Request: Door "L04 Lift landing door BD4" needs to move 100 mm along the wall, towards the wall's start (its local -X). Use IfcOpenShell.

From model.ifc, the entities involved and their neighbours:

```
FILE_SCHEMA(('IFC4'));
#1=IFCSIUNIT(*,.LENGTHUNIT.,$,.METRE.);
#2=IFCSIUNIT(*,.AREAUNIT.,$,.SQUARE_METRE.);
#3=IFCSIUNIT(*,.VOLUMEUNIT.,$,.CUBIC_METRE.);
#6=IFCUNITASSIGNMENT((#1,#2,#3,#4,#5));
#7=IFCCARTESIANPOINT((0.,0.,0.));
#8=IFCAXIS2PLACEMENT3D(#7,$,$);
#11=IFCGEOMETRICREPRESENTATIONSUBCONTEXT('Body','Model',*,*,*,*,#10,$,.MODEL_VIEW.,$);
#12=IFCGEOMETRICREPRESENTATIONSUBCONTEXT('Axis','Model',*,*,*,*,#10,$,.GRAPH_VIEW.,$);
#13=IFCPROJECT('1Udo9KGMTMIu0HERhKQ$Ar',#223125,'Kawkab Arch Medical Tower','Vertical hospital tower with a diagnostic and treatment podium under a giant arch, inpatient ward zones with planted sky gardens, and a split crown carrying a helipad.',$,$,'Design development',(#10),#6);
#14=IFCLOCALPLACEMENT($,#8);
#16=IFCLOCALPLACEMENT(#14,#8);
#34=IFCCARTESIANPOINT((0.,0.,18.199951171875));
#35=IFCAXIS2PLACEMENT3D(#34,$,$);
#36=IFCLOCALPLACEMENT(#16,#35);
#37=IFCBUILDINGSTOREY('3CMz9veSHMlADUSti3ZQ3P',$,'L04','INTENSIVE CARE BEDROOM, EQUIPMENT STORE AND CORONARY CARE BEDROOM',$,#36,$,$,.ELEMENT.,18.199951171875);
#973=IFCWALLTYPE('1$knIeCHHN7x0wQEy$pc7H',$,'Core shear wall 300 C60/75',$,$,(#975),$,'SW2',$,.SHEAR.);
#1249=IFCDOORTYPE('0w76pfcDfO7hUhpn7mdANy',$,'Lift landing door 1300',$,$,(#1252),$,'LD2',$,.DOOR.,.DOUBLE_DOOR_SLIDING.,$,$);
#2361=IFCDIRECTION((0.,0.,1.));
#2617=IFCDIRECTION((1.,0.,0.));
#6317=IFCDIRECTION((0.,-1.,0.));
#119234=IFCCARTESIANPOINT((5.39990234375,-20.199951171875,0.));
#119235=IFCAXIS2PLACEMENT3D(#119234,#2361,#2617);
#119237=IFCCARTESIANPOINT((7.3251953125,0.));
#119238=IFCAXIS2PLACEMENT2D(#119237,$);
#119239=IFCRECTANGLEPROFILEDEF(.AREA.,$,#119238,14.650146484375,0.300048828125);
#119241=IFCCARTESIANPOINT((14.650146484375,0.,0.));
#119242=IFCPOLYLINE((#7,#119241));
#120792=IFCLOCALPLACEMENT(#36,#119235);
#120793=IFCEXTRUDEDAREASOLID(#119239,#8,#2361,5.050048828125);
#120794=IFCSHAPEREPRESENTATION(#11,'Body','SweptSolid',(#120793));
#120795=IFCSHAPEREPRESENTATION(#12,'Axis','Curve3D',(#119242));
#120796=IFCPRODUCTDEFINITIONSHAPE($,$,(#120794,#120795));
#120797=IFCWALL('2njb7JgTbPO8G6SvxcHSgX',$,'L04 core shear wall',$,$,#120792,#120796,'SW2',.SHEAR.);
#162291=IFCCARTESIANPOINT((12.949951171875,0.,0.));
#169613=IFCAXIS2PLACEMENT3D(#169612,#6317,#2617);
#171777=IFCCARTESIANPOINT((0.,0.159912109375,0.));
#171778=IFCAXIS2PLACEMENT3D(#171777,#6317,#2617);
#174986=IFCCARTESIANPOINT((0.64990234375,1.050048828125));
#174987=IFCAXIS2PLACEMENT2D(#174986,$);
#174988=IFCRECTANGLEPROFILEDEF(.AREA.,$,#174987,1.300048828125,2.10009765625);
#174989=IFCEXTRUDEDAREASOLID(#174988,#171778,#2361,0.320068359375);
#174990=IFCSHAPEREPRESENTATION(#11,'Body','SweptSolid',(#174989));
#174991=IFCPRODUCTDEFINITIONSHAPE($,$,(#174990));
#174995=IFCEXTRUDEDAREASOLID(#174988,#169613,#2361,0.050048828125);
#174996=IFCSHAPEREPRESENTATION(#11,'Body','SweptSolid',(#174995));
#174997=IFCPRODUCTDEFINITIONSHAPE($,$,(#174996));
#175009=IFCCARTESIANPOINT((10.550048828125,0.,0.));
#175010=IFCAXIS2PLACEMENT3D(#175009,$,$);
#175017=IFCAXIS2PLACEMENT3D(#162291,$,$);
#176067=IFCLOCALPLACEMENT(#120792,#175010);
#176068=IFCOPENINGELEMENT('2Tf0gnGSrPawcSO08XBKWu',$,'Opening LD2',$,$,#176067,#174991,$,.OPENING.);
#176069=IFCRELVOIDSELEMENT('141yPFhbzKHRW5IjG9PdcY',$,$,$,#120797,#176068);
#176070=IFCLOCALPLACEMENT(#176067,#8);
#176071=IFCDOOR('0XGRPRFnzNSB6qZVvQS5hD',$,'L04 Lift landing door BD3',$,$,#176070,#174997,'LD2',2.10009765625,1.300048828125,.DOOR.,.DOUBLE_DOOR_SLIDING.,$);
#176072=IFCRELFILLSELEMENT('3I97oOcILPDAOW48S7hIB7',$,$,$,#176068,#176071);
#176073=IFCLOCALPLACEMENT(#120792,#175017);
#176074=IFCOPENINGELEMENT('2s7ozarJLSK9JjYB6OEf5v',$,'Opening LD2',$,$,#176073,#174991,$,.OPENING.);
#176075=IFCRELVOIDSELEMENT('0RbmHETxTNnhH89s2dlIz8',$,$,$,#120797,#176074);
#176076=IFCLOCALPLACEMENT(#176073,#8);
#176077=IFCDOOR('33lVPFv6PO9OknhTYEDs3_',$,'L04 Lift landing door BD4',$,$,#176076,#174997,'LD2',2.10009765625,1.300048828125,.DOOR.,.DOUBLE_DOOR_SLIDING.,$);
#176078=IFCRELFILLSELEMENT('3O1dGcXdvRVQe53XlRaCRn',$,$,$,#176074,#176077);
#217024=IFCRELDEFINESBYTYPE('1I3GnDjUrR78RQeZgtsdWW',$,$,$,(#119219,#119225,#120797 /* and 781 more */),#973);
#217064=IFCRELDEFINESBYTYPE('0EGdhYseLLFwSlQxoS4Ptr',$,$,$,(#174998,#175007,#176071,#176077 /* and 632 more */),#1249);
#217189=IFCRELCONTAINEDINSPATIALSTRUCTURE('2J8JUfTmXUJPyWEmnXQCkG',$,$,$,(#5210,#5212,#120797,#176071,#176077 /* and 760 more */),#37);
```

```python
import ifcopenshell
import ifcopenshell.api.geometry
import ifcopenshell.util.placement

model = ifcopenshell.open("model.ifc")

door = model.by_id(176077)
opening = door.FillsVoids[0].RelatingOpeningElement
wall = opening.VoidsElements[0].RelatingBuildingElement

wall_matrix = ifcopenshell.util.placement.get_local_placement(wall.ObjectPlacement)
shift = wall_matrix[:3, 0] * -0.1
before = ifcopenshell.util.placement.get_local_placement(door.ObjectPlacement)[:3, 3].copy()

# The door is placed relative to its opening, so it follows when the opening moves.
matrix = ifcopenshell.util.placement.get_local_placement(opening.ObjectPlacement)
matrix[:3, 3] += shift
ifcopenshell.api.geometry.edit_object_placement(
    model, product=opening, matrix=matrix, is_si=False, should_transform_children=True
)

after = ifcopenshell.util.placement.get_local_placement(door.ObjectPlacement)[:3, 3]
print("door moved by", (after - before).round(3) + 0.0)

model.write("model_updated.ifc")
```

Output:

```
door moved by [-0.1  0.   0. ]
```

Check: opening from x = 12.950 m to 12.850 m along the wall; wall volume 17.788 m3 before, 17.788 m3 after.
